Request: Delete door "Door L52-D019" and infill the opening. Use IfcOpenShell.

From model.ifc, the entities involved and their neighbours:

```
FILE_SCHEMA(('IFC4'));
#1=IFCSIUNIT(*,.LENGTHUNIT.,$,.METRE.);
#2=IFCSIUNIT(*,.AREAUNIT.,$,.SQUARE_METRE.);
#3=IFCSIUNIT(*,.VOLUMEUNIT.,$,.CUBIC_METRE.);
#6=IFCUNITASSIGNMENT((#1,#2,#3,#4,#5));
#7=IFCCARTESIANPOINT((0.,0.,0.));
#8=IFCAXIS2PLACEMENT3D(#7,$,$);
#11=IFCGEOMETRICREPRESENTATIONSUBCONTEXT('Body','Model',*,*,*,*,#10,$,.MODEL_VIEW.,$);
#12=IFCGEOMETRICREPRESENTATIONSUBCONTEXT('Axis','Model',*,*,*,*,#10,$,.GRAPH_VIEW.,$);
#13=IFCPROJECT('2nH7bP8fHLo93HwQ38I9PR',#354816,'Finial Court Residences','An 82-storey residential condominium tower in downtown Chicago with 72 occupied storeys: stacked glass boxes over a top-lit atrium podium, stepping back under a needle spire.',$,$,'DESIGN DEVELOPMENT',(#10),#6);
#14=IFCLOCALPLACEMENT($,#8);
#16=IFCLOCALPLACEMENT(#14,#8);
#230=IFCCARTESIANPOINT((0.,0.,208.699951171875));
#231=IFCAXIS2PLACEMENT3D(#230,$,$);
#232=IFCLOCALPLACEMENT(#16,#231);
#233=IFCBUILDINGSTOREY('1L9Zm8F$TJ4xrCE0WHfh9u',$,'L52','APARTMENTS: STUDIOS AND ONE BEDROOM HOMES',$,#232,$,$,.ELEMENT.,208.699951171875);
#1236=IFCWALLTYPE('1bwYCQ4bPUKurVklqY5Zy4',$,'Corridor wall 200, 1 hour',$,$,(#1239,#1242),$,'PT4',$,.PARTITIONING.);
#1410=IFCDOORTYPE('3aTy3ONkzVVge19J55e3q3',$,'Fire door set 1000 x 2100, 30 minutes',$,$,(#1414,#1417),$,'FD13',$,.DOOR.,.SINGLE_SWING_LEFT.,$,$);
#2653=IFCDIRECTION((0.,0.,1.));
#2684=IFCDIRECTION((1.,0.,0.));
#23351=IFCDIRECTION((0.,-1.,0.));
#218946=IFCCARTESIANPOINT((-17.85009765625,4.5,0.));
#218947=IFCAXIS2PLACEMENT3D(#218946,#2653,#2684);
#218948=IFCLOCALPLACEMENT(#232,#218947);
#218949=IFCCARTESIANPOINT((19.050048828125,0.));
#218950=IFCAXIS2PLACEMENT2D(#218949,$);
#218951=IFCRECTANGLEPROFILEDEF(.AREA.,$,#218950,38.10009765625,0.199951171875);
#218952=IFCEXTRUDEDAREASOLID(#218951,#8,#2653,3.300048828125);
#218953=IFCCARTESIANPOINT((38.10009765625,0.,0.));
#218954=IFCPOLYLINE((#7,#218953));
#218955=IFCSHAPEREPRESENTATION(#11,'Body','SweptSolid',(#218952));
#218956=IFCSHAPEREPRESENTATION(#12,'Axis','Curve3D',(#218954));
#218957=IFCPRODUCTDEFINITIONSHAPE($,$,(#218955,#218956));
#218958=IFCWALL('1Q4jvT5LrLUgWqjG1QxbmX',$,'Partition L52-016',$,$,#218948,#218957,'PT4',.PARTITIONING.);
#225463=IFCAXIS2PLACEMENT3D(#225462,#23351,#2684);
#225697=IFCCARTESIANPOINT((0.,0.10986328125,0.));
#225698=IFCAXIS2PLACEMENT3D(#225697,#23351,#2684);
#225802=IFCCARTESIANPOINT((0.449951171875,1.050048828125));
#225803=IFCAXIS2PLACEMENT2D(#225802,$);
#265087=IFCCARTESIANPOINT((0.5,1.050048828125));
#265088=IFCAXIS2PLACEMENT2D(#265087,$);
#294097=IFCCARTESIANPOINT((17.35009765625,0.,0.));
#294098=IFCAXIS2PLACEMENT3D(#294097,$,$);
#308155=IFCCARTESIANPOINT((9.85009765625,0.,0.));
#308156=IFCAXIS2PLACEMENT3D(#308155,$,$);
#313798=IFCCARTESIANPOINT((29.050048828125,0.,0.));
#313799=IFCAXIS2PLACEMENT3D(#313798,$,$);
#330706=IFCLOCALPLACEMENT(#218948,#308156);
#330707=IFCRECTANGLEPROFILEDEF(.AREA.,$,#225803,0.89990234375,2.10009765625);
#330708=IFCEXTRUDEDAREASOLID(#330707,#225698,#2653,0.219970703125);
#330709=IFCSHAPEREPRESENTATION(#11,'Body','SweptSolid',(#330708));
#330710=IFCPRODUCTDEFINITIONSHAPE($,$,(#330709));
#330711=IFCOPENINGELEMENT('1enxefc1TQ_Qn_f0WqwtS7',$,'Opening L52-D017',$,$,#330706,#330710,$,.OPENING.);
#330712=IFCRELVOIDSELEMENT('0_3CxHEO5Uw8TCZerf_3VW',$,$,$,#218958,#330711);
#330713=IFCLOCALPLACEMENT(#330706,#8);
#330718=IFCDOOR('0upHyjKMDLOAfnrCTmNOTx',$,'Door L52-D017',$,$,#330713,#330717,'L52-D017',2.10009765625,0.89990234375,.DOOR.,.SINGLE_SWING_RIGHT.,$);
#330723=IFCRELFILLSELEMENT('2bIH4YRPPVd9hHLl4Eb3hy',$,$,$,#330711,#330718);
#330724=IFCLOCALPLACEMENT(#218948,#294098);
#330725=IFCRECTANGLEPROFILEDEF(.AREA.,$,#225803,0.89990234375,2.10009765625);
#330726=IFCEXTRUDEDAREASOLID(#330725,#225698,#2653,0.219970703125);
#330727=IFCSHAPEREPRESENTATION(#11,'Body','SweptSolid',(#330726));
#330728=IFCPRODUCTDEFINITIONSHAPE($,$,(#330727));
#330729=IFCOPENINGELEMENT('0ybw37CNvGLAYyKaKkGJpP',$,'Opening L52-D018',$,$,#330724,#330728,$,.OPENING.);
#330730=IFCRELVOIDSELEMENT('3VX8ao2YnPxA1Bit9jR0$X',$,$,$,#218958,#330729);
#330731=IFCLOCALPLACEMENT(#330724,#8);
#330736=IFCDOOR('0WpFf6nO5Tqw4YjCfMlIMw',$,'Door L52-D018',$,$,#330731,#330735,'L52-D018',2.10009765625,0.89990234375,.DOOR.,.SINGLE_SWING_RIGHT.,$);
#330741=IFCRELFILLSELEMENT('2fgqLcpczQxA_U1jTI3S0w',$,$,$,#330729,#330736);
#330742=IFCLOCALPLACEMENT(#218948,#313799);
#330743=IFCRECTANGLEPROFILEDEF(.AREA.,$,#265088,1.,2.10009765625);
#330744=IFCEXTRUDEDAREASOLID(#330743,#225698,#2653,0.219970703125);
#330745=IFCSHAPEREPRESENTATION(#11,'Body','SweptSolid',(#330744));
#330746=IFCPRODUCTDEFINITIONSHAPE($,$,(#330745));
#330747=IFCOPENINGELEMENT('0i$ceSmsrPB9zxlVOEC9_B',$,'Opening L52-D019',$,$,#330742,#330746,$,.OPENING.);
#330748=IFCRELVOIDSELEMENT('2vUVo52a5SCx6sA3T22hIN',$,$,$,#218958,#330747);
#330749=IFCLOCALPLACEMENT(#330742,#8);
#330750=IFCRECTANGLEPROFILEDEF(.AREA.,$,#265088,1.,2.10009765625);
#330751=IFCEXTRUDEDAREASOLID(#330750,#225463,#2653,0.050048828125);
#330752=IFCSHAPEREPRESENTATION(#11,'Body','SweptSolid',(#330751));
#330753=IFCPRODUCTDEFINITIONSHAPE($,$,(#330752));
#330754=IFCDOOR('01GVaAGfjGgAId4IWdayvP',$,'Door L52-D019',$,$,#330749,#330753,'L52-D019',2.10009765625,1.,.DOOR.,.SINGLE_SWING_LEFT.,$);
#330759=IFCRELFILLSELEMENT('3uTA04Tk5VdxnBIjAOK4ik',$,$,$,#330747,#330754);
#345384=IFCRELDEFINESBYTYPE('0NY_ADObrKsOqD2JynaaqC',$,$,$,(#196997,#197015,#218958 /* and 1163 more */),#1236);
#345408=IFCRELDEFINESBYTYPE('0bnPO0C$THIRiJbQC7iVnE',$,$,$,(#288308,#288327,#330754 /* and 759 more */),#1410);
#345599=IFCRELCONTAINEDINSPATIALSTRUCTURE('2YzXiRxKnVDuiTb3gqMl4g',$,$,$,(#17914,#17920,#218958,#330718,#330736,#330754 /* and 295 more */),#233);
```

```python
import ifcopenshell
import ifcopenshell.api.feature
import ifcopenshell.api.root
import ifcopenshell.geom
import ifcopenshell.util.shape

model = ifcopenshell.open("model.ifc")
settings = ifcopenshell.geom.settings()


def volume(element):
    """Net volume in cubic metres, openings subtracted."""
    shape = ifcopenshell.geom.create_shape(settings, element)
    return ifcopenshell.util.shape.get_volume(shape.geometry)


door = model.by_id(330754)
opening = door.FillsVoids[0].RelatingOpeningElement
wall = opening.VoidsElements[0].RelatingBuildingElement
before = volume(wall)

ifcopenshell.api.root.remove_product(model, product=door)
ifcopenshell.api.feature.remove_feature(model, feature=opening)

after = volume(wall)

print(f"wall volume {before:.3f} -> {after:.3f} m3")

model.write("model-out.ifc")
```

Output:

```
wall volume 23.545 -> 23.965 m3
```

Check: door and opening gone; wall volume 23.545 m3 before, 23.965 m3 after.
